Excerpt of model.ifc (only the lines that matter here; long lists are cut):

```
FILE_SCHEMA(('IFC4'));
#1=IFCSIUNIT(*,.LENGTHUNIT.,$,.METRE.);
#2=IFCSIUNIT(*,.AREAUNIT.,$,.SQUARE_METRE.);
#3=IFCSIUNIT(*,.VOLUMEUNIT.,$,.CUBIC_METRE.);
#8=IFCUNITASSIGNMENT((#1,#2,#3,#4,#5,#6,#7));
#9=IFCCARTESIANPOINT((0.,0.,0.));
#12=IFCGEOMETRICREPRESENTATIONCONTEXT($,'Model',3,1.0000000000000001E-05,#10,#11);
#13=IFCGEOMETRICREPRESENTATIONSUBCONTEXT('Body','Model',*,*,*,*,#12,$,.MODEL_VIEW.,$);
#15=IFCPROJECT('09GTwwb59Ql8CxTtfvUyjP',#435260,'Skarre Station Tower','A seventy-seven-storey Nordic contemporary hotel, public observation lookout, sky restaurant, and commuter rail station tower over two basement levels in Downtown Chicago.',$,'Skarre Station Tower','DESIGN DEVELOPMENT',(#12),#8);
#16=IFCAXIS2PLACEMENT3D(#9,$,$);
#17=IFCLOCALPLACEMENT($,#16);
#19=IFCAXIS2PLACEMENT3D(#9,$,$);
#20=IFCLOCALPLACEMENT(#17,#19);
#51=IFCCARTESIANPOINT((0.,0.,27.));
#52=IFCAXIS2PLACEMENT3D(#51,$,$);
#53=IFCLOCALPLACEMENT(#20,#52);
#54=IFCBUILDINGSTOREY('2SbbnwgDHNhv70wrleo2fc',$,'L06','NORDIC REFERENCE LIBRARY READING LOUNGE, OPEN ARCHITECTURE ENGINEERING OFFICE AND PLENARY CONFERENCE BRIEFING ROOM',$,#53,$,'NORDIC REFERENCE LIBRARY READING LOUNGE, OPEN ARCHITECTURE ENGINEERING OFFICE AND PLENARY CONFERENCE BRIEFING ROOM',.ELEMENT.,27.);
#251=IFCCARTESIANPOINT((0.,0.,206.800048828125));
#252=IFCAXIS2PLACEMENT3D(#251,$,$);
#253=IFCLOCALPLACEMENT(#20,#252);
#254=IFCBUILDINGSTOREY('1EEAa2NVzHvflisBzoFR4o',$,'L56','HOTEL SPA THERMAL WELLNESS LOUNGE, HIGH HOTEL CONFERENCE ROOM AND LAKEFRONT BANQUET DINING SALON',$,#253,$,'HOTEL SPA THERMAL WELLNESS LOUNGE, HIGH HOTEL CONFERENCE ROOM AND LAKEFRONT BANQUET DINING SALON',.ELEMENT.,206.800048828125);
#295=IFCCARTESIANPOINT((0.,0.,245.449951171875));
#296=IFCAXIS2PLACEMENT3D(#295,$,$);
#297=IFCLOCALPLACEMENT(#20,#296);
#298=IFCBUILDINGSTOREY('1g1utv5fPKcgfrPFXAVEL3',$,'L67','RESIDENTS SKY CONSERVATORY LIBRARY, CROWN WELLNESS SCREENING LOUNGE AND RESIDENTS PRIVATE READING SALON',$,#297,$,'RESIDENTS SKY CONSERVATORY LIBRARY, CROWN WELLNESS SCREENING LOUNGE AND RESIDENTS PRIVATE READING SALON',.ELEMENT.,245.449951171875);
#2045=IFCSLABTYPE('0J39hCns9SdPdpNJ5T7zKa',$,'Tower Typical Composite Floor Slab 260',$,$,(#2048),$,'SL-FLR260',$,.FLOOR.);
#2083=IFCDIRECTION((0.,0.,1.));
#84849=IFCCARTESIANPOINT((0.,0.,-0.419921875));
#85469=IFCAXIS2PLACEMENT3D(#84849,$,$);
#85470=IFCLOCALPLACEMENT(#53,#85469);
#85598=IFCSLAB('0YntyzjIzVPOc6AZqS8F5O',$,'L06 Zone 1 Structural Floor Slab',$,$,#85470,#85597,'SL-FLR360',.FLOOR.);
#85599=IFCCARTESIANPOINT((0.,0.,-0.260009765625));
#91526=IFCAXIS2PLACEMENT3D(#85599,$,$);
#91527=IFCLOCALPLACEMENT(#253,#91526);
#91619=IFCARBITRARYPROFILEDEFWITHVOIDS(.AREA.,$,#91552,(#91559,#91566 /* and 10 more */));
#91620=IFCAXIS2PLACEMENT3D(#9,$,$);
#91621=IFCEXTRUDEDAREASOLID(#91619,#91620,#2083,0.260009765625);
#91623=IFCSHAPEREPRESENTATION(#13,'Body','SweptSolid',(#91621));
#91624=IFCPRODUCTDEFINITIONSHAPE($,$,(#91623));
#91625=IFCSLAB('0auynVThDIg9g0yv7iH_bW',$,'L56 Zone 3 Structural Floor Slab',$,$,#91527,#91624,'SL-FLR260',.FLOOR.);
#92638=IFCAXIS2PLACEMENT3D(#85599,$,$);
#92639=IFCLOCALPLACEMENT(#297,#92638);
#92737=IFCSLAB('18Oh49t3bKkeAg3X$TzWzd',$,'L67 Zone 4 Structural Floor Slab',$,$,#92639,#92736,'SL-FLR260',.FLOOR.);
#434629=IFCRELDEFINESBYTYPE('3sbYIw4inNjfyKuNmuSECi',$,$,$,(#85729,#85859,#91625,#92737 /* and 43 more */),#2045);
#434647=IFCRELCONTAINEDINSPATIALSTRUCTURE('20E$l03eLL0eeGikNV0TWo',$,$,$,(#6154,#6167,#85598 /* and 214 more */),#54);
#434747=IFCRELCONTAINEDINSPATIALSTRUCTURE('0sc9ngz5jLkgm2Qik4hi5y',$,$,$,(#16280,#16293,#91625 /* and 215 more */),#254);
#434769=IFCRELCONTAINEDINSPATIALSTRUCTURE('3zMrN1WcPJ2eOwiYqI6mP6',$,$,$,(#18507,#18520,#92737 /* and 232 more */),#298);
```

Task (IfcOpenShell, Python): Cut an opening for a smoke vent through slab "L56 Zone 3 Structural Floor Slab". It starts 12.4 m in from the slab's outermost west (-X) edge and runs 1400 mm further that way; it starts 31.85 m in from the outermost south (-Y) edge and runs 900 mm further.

```python
import numpy as np
import ifcopenshell
import ifcopenshell.api.feature
import ifcopenshell.api.geometry
import ifcopenshell.api.root
import ifcopenshell.geom
import ifcopenshell.util.placement
import ifcopenshell.util.representation
import ifcopenshell.util.shape
import ifcopenshell.util.unit

model = ifcopenshell.open("model.ifc")
unit_scale = ifcopenshell.util.unit.calculate_unit_scale(model)
settings = ifcopenshell.geom.settings()


def volume(element):
    """Net volume in cubic metres, openings subtracted."""
    shape = ifcopenshell.geom.create_shape(settings, element)
    return ifcopenshell.util.shape.get_volume(shape.geometry)


slab = model.by_guid("0auynVThDIg9g0yv7iH_bW")
before = volume(slab)

# Extent in the slab's own axes, in metres. The edges named are its -X and -Y sides.
slab_shape = ifcopenshell.geom.create_shape(settings, slab)
vertices = ifcopenshell.util.shape.get_vertices(slab_shape.geometry)
x_min, y_min, bottom = vertices.min(axis=0)
top = vertices[:, 2].max()

opening = ifcopenshell.api.root.create_entity(model, ifc_class="IfcOpeningElement", name="Smoke vent opening", predefined_type="OPENING")
context = ifcopenshell.util.representation.get_context(model, "Model", "Body", "MODEL_VIEW")
width, depth = 1.4, 0.9
outline = [(0.0, 0.0), (width, 0.0), (width, depth), (0.0, depth), (0.0, 0.0)]
# Overshoot both faces by 50 mm so the cut is clean.
shape = ifcopenshell.api.geometry.add_slab_representation(
    model, context=context, depth=top - bottom + 0.1, polyline=outline
)
ifcopenshell.api.geometry.assign_representation(model, product=opening, representation=shape)

matrix = ifcopenshell.util.placement.get_local_placement(slab.ObjectPlacement)
matrix[:, 3] = matrix @ np.append(np.array([x_min + 12.4, y_min + 31.85, bottom - 0.05]) / unit_scale, 1.0)
ifcopenshell.api.geometry.edit_object_placement(model, product=opening, matrix=matrix, is_si=False)
ifcopenshell.api.feature.add_feature(model, feature=opening, element=slab)

after = volume(slab)

print(f"slab volume {before:.3f} -> {after:.3f} m3")

model.write("model_updated.ifc")
```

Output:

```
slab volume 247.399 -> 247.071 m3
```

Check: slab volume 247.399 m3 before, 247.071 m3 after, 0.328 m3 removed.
